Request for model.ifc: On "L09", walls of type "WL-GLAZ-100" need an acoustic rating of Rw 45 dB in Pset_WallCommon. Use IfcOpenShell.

First a look at what the model holds.

```python
import ifcopenshell
import ifcopenshell.util.element

model = ifcopenshell.open("model.ifc")
print(model.schema)
storey = next(s for s in model.by_type("IfcBuildingStorey") if s.Name == "L09")
walls = [e for e in ifcopenshell.util.element.get_decomposition(storey) if e.is_a("IfcWall")]
seen = {}
for e in walls:
    element_type = ifcopenshell.util.element.get_type(e)
    key = (element_type.Name if element_type != e and element_type else None, ifcopenshell.util.element.get_pset(e, "Pset_WallCommon", "AcousticRating"))
    seen[key] = seen.get(key, 0) + 1
for (name, value), count in sorted(seen.items(), key=str):
    print(count, "x", name, "|", value)
```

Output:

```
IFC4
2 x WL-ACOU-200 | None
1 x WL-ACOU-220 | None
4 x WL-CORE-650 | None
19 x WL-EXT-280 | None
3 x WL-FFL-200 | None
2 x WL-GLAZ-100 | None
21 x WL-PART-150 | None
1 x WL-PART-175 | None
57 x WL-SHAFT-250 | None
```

```python
import ifcopenshell
import ifcopenshell.api.pset
import ifcopenshell.util.element

model = ifcopenshell.open("model.ifc")

storey = next(s for s in model.by_type("IfcBuildingStorey") if s.Name == "L09")
walls = [e for e in ifcopenshell.util.element.get_decomposition(storey) if e.is_a("IfcWall")]

count = 0
for e in walls:
    element_type = ifcopenshell.util.element.get_type(e)
    if element_type in (None, e) or element_type.Name != "WL-GLAZ-100":
        continue
    # add_pset returns the element's existing set when there is one.
    pset = ifcopenshell.api.pset.add_pset(model, product=e, name="Pset_WallCommon")
    ifcopenshell.api.pset.edit_pset(model, pset=pset, properties={"AcousticRating": "Rw 45 dB"})
    count += 1

print(count, "walls updated")

model.write("model_v2.ifc")
```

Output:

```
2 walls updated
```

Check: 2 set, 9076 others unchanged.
